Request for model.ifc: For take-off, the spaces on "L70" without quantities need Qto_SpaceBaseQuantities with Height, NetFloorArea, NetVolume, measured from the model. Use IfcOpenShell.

First a look at what the model holds.

```python
import ifcopenshell
import ifcopenshell.util.element
import ifcopenshell.util.unit

model = ifcopenshell.open("model.ifc")
print(model.schema)
for unit_type in ("LENGTHUNIT", "AREAUNIT", "VOLUMEUNIT"):
    print(unit_type, ifcopenshell.util.unit.calculate_unit_scale(model, unit_type))
storey = next(s for s in model.by_type("IfcBuildingStorey") if s.Name == "L70")
spaces = [e for e in ifcopenshell.util.element.get_decomposition(storey) if e.is_a("IfcSpace")]
for e in sorted(spaces, key=lambda e: e.id()):
    print(e.id(), e.is_a(), e.Name, list(ifcopenshell.util.element.get_psets(e, qtos_only=True)), sep=" | ")
```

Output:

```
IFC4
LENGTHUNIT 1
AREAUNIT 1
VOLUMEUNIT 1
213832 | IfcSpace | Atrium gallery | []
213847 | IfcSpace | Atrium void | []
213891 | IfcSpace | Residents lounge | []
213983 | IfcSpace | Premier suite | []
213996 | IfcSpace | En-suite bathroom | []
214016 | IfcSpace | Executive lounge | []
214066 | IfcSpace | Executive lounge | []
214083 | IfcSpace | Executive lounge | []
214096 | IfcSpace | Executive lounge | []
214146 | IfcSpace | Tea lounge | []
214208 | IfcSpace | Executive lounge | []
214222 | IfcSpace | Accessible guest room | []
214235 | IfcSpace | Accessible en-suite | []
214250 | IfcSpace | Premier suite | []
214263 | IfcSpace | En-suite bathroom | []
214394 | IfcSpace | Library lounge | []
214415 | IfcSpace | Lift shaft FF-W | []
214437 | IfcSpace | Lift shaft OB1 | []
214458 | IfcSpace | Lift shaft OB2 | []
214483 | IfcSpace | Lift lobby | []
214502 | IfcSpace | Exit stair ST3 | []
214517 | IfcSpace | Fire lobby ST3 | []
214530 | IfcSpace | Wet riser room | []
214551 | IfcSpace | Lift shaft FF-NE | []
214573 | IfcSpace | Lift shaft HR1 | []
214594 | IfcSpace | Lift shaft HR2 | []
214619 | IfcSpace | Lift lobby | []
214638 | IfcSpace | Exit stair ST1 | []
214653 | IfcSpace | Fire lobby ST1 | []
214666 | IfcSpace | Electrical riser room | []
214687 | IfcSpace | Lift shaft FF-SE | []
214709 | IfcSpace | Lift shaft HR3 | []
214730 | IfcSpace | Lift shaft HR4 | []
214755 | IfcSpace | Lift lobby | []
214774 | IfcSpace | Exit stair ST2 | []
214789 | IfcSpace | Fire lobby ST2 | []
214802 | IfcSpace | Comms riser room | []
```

```python
import ifcopenshell
import ifcopenshell.api.pset
import ifcopenshell.geom
import ifcopenshell.util.element
import ifcopenshell.util.shape
import ifcopenshell.util.unit

model = ifcopenshell.open("model.ifc")
unit_scale = ifcopenshell.util.unit.calculate_unit_scale(model)
area_scale = ifcopenshell.util.unit.calculate_unit_scale(model, "AREAUNIT")
volume_scale = ifcopenshell.util.unit.calculate_unit_scale(model, "VOLUMEUNIT")
settings = ifcopenshell.geom.settings()

storey = next(s for s in model.by_type("IfcBuildingStorey") if s.Name == "L70")
spaces = [e for e in ifcopenshell.util.element.get_decomposition(storey) if e.is_a("IfcSpace")]

for e in sorted(spaces, key=lambda e: e.id()):
    if ifcopenshell.util.element.get_psets(e, qtos_only=True, should_inherit=False):
        continue
    # Geometry comes back in metres, in the element's own axes.
    shape = ifcopenshell.geom.create_shape(settings, e)
    values = {
        "Height": ifcopenshell.util.shape.get_z(shape.geometry) / unit_scale,
        "NetFloorArea": ifcopenshell.util.shape.get_footprint_area(shape.geometry) / area_scale,
        "NetVolume": ifcopenshell.util.shape.get_volume(shape.geometry) / volume_scale,
    }
    qto = ifcopenshell.api.pset.add_qto(model, product=e, name="Qto_SpaceBaseQuantities")
    ifcopenshell.api.pset.edit_qto(model, qto=qto, properties=values)
    print(e.id(), {k: round(v, 3) for k, v in values.items()})

model.write("model_edited.ifc")
```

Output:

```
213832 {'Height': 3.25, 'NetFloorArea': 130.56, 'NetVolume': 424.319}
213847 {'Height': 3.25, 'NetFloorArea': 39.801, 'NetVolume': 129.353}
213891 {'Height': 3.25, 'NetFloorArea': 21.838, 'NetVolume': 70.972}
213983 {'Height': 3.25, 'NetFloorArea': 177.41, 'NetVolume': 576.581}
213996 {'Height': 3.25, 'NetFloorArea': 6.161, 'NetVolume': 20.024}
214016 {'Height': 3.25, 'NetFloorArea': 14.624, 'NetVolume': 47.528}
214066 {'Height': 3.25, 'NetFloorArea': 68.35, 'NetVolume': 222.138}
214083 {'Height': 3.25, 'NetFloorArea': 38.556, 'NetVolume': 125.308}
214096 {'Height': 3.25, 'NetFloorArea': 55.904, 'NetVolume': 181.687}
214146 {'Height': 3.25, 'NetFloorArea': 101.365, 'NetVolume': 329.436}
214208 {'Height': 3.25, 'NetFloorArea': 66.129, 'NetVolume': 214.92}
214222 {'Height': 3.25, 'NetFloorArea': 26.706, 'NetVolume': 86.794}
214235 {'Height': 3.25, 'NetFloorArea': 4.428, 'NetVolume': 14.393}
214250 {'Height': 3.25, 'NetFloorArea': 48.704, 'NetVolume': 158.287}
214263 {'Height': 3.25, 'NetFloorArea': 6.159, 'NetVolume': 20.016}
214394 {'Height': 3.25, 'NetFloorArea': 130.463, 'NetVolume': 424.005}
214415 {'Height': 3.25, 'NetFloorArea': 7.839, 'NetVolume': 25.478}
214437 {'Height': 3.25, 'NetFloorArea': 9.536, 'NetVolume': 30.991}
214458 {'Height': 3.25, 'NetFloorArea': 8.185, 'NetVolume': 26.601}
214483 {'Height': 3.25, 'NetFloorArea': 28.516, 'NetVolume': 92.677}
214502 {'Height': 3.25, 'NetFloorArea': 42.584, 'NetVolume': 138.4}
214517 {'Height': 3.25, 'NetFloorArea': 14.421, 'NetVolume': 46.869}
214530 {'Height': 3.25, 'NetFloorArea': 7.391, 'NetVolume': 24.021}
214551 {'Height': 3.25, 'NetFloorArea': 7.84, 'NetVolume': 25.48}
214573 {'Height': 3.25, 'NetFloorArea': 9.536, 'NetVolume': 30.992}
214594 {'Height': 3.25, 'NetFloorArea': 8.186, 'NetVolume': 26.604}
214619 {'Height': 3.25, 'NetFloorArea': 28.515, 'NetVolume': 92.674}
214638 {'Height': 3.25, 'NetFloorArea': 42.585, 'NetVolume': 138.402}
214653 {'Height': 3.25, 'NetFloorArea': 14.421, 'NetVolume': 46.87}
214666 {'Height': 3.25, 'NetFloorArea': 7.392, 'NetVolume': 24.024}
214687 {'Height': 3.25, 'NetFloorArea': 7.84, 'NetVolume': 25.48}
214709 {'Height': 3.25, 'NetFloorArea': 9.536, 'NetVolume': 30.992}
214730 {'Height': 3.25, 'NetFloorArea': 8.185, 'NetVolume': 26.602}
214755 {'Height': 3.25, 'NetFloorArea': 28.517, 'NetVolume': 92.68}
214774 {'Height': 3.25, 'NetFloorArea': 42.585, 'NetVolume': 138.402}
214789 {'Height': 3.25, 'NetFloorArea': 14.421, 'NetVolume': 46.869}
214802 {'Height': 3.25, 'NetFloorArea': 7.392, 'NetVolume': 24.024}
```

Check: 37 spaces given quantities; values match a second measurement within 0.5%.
